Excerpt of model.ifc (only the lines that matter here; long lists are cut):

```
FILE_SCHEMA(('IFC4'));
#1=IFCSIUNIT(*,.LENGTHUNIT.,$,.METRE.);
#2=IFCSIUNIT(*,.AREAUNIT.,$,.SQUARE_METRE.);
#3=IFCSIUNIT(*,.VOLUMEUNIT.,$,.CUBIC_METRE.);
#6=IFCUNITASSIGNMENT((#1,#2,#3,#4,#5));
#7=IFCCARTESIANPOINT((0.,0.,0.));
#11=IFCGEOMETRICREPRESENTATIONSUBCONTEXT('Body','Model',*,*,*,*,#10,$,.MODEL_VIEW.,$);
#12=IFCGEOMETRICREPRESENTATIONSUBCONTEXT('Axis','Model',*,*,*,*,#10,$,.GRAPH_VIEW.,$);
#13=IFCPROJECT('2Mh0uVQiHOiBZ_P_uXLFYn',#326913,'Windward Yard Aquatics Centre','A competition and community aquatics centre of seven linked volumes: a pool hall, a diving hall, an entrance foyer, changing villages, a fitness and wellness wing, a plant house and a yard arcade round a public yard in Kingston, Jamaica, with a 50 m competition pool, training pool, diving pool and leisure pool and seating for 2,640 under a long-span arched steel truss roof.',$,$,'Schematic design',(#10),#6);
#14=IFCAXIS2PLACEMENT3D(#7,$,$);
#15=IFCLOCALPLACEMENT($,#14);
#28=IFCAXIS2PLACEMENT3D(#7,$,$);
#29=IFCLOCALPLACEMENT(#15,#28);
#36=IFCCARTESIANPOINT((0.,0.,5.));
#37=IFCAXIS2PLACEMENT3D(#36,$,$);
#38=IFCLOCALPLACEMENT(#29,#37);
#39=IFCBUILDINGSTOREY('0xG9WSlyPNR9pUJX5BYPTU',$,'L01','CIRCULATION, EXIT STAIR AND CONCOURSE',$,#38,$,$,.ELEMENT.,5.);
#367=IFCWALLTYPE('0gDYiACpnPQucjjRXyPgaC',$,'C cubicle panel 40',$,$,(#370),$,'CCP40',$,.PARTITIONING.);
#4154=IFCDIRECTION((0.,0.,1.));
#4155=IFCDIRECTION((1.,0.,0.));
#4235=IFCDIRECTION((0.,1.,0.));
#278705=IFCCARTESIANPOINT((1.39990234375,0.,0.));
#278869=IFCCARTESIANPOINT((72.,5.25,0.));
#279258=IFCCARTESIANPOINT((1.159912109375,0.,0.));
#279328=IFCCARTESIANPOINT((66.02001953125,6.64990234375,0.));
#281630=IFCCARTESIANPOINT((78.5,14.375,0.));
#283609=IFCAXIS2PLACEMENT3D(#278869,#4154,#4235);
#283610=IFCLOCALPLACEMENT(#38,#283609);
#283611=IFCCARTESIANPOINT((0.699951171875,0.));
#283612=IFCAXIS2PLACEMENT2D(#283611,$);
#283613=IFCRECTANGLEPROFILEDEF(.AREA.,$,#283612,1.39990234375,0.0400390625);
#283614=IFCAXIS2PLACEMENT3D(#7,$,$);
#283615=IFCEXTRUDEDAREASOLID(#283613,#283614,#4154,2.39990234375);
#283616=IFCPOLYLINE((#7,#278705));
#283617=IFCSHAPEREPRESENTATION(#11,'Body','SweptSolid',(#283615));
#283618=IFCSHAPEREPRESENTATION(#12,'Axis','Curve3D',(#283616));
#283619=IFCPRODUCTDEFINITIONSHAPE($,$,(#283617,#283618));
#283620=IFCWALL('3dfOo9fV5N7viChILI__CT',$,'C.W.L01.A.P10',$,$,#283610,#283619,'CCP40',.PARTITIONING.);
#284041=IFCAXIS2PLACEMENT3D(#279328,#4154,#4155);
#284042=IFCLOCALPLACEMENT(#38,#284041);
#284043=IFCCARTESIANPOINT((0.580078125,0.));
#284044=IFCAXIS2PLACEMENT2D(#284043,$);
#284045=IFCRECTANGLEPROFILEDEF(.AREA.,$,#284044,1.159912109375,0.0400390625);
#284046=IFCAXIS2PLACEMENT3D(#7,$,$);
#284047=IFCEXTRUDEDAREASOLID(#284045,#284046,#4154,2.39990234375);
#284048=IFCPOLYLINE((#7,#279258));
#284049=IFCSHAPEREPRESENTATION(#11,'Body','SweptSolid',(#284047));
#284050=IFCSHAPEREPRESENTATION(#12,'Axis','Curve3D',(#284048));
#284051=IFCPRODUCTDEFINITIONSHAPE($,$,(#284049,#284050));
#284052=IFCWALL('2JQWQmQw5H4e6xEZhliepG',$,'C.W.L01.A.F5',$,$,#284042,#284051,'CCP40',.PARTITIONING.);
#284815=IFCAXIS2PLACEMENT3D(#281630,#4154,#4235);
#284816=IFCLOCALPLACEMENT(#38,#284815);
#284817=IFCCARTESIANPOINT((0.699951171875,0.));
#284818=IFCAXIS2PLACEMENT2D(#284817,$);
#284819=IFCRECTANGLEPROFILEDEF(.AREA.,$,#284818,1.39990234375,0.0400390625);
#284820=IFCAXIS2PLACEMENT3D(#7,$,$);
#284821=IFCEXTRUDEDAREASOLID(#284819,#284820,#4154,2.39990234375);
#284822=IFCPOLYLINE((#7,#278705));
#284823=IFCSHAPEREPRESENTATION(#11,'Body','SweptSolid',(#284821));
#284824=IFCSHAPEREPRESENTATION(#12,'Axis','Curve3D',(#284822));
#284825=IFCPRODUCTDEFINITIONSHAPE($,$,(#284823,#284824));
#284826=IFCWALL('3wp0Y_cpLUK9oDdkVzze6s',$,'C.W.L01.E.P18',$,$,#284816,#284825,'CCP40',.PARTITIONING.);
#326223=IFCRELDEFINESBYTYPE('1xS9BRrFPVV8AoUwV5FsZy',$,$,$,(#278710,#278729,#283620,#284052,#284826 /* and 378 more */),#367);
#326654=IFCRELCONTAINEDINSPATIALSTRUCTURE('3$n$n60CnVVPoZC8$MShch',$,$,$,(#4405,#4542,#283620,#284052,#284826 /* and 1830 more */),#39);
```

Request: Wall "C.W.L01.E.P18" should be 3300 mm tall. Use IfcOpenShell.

```python
import ifcopenshell
import ifcopenshell.geom
import ifcopenshell.util.representation
import ifcopenshell.util.shape
import ifcopenshell.util.unit

model = ifcopenshell.open("model.ifc")
unit_scale = ifcopenshell.util.unit.calculate_unit_scale(model)
settings = ifcopenshell.geom.settings()


def volume(element):
    """Net volume in cubic metres, openings subtracted."""
    shape = ifcopenshell.geom.create_shape(settings, element)
    return ifcopenshell.util.shape.get_volume(shape.geometry)


wall = model.by_guid("3wp0Y_cpLUK9oDdkVzze6s")
before = volume(wall)

body = ifcopenshell.util.representation.get_representation(wall, "Model", "Body")
solid = body.Items[0]
old_height = solid.Depth
solid.Depth = 3.3 / unit_scale
after = volume(wall)

print(f"height {old_height:g} -> {solid.Depth:g}, volume {before:.3f} -> {after:.3f} m3")

model.write("model_v2.ifc")
```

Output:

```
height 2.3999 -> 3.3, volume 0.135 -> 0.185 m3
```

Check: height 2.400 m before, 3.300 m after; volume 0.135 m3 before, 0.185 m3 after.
